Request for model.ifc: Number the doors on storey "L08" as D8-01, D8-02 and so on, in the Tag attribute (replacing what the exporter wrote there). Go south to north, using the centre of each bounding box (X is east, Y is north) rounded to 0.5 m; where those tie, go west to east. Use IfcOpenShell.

First a look at what the model holds.

```python
import ifcopenshell
import ifcopenshell.util.element
import ifcopenshell.util.placement

model = ifcopenshell.open("model.ifc")
print(model.schema)
storey = next(s for s in model.by_type("IfcBuildingStorey") if s.Name == "L08")
doors = [e for e in ifcopenshell.util.element.get_decomposition(storey) if e.is_a("IfcDoor")]
for e in sorted(doors, key=lambda e: e.id()):
    origin = ifcopenshell.util.placement.get_local_placement(e.ObjectPlacement)[:3, 3]
    print(e.id(), e.Tag, e.Name, origin.round(2) + 0.0, sep=" | ")
```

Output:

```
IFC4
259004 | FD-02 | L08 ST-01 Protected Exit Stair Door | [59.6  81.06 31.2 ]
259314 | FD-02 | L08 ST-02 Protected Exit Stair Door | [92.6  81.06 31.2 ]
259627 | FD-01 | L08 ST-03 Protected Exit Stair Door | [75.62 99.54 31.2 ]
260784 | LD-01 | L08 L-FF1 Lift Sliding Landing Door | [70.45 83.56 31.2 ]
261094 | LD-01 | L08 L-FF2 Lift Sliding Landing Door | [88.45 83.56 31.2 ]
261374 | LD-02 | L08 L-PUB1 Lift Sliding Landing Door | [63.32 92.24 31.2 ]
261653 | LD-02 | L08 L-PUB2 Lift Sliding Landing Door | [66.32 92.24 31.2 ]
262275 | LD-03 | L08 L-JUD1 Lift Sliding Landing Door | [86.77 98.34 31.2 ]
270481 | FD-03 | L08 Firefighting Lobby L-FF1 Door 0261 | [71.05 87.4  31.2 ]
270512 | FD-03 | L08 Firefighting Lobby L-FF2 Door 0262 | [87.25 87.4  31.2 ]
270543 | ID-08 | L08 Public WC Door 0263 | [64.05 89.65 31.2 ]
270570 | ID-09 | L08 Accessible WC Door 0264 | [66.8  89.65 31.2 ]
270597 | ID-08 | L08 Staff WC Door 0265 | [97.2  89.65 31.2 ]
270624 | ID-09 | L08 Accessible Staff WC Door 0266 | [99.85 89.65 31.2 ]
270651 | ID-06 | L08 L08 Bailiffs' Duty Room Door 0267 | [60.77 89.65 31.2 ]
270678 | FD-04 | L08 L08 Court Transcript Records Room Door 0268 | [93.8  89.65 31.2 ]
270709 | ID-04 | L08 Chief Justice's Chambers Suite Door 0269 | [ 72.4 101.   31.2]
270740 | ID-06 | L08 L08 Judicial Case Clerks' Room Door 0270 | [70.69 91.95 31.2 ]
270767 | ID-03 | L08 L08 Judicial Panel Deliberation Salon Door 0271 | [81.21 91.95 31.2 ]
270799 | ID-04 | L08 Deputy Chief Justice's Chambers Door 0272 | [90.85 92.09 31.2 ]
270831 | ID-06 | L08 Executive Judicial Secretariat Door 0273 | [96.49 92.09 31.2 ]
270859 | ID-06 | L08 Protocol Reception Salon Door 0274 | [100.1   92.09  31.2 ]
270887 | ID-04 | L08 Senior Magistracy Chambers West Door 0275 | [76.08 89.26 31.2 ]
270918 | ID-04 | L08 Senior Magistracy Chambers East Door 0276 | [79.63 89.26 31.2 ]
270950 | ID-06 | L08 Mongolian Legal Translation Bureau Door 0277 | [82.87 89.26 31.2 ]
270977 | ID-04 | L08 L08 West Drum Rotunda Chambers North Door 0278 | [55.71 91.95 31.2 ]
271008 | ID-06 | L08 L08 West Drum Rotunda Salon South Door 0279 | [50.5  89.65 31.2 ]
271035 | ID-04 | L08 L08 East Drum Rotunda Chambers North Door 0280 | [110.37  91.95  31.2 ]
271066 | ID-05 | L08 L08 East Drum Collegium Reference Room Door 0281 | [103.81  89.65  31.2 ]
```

```python
import ifcopenshell
import ifcopenshell.geom
import ifcopenshell.util.element
import ifcopenshell.util.shape

model = ifcopenshell.open("model.ifc")
settings = ifcopenshell.geom.settings()
settings.set("use-world-coords", True)


def centre(element):
    shape = ifcopenshell.geom.create_shape(settings, element)
    return ifcopenshell.util.shape.get_bbox_centroid(shape.geometry)


storey = next(s for s in model.by_type("IfcBuildingStorey") if s.Name == "L08")
doors = [e for e in ifcopenshell.util.element.get_decomposition(storey) if e.is_a("IfcDoor")]

# Insertion points can sit at a corner or the storey origin, so sort by the geometry (in metres).
centres = {e: centre(e) for e in doors}
doors.sort(key=lambda e: (round(centres[e][1] / 0.5), centres[e][0]))

for i, e in enumerate(doors, start=1):
    number = f"D8-{i:02d}"
    e.Tag = number
    print(e.id(), number)

model.write("model_edited.ifc")
```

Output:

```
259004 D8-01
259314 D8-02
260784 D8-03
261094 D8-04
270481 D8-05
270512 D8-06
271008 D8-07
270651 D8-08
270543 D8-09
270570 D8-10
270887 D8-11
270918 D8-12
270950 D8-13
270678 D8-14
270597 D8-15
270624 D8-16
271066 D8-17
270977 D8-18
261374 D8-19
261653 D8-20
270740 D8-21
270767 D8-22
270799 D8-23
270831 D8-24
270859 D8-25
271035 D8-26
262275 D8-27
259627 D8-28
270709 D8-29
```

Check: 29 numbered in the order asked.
